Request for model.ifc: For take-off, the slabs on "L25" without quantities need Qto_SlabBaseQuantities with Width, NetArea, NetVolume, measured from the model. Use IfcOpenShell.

First a look at what the model holds.

```python
import ifcopenshell
import ifcopenshell.util.element
import ifcopenshell.util.unit

model = ifcopenshell.open("model.ifc")
print(model.schema)
for unit_type in ("LENGTHUNIT", "AREAUNIT", "VOLUMEUNIT"):
    print(unit_type, ifcopenshell.util.unit.calculate_unit_scale(model, unit_type))
storey = next(s for s in model.by_type("IfcBuildingStorey") if s.Name == "L25")
slabs = [e for e in ifcopenshell.util.element.get_decomposition(storey) if e.is_a("IfcSlab")]
for e in sorted(slabs, key=lambda e: e.id()):
    print(e.id(), e.is_a(), e.Name, list(ifcopenshell.util.element.get_psets(e, qtos_only=True)), sep=" | ")
```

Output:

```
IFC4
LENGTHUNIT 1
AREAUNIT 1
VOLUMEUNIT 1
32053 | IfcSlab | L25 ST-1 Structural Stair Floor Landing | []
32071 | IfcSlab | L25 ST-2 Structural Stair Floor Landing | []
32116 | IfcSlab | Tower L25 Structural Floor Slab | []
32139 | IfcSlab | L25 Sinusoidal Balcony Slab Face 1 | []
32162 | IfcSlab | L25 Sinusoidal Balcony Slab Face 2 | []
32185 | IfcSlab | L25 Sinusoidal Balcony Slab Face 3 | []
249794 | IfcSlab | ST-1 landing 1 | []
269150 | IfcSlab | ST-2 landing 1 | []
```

```python
import ifcopenshell
import ifcopenshell.api.pset
import ifcopenshell.geom
import ifcopenshell.util.element
import ifcopenshell.util.shape
import ifcopenshell.util.unit

model = ifcopenshell.open("model.ifc")
unit_scale = ifcopenshell.util.unit.calculate_unit_scale(model)
area_scale = ifcopenshell.util.unit.calculate_unit_scale(model, "AREAUNIT")
volume_scale = ifcopenshell.util.unit.calculate_unit_scale(model, "VOLUMEUNIT")
settings = ifcopenshell.geom.settings()

storey = next(s for s in model.by_type("IfcBuildingStorey") if s.Name == "L25")
slabs = [e for e in ifcopenshell.util.element.get_decomposition(storey) if e.is_a("IfcSlab")]

for e in sorted(slabs, key=lambda e: e.id()):
    if ifcopenshell.util.element.get_psets(e, qtos_only=True, should_inherit=False):
        continue
    # Geometry comes back in metres, in the element's own axes.
    shape = ifcopenshell.geom.create_shape(settings, e)
    values = {
        "Width": ifcopenshell.util.shape.get_z(shape.geometry) / unit_scale,
        "NetArea": ifcopenshell.util.shape.get_footprint_area(shape.geometry) / area_scale,
        "NetVolume": ifcopenshell.util.shape.get_volume(shape.geometry) / volume_scale,
    }
    qto = ifcopenshell.api.pset.add_qto(model, product=e, name="Qto_SlabBaseQuantities")
    ifcopenshell.api.pset.edit_qto(model, qto=qto, properties=values)
    print(e.id(), {k: round(v, 3) for k, v in values.items()})

model.write("model_rev.ifc")
```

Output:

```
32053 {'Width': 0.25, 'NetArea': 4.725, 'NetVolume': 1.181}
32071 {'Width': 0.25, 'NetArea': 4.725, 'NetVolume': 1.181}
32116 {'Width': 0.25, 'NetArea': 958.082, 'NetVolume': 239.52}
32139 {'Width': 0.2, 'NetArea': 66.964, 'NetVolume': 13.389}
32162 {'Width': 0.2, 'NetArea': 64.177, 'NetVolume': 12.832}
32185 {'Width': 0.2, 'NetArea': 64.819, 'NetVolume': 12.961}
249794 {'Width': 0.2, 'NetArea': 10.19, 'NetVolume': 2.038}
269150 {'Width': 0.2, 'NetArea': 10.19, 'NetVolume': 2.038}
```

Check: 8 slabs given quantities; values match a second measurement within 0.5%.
